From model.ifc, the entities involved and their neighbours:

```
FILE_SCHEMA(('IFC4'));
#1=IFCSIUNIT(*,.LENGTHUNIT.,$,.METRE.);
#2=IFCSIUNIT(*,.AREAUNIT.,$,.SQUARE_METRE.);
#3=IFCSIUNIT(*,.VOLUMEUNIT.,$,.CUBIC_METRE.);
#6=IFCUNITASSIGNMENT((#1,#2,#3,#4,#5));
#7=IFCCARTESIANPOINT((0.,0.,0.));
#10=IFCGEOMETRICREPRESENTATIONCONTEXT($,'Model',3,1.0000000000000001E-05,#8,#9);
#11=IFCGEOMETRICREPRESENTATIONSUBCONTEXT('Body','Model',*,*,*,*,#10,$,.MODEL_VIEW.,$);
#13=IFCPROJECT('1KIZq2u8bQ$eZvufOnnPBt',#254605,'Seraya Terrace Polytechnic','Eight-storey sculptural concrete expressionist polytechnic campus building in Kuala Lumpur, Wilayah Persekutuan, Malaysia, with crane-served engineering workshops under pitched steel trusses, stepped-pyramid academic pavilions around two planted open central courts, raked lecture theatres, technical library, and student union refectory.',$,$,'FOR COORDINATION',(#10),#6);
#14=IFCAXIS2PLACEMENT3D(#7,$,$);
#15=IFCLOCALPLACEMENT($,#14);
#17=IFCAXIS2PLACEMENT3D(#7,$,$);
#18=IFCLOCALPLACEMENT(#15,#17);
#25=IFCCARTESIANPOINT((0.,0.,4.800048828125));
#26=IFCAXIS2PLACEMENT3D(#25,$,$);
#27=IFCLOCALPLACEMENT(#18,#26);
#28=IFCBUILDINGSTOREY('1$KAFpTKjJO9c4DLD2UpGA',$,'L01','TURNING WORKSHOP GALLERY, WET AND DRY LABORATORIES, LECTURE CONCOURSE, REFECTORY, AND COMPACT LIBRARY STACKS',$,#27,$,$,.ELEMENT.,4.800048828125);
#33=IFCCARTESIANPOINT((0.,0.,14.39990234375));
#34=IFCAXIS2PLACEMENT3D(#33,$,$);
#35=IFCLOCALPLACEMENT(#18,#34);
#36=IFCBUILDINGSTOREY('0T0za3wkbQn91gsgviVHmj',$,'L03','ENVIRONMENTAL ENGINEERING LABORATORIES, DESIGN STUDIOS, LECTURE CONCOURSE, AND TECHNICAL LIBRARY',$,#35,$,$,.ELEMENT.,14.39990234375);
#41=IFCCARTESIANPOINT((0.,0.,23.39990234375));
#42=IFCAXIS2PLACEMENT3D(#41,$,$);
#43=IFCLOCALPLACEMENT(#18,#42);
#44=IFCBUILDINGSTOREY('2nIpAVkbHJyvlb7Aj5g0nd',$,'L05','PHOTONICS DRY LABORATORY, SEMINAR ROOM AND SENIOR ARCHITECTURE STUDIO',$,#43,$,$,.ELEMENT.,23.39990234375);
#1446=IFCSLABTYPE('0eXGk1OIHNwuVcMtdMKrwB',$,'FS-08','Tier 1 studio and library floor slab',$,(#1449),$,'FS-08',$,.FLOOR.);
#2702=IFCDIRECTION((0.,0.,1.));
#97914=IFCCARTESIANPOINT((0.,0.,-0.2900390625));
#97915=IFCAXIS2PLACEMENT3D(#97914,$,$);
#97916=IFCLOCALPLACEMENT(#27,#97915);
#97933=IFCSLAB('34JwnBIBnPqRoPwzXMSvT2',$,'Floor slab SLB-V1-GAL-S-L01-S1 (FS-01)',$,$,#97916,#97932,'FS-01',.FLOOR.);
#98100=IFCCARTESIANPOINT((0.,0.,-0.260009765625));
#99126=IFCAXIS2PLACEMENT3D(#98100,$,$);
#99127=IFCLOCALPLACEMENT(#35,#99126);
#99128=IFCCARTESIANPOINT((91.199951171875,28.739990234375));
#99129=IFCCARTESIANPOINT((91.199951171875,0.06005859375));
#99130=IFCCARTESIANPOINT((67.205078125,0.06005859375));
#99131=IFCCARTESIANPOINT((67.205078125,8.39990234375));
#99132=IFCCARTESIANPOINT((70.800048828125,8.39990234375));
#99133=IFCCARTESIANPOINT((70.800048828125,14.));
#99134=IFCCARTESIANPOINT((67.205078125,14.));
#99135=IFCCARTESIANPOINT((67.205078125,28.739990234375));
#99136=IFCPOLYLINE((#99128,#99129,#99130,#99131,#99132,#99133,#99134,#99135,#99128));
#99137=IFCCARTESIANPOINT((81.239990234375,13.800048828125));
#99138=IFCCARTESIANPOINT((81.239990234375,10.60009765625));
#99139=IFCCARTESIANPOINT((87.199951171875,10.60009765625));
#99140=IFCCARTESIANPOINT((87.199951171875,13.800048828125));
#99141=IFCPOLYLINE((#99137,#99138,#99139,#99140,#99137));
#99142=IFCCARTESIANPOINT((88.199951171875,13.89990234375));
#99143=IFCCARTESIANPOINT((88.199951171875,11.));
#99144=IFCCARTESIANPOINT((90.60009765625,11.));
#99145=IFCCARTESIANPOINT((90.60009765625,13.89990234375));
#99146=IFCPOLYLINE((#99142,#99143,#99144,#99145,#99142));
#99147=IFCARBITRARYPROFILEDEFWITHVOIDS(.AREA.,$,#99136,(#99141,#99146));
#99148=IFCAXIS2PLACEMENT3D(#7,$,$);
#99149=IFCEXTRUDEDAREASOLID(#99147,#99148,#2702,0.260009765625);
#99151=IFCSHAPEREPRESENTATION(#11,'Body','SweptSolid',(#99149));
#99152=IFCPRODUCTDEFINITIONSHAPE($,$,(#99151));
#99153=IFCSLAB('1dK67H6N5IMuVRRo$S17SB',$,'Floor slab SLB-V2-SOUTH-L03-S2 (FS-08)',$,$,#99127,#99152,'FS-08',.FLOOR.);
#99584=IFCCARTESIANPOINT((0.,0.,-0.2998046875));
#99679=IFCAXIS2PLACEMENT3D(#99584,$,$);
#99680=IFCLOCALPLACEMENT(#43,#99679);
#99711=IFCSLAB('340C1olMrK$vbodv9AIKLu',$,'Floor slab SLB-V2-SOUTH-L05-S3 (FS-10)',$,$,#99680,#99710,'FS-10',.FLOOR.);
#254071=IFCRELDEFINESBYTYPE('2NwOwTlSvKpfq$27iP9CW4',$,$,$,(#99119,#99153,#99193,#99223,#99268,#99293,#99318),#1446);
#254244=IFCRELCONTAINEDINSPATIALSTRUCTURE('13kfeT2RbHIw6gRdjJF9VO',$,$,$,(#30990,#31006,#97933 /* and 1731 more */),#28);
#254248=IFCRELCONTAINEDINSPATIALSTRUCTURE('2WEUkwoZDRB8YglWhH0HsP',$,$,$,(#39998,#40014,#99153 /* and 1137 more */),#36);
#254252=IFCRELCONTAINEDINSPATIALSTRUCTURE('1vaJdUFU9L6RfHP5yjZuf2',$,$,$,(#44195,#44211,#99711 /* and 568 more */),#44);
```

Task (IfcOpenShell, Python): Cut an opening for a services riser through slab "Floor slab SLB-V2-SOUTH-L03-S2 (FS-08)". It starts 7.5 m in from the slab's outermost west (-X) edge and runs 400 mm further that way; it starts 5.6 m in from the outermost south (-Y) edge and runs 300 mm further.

```python
import numpy as np
import ifcopenshell
import ifcopenshell.api.feature
import ifcopenshell.api.geometry
import ifcopenshell.api.root
import ifcopenshell.geom
import ifcopenshell.util.placement
import ifcopenshell.util.representation
import ifcopenshell.util.shape
import ifcopenshell.util.unit

model = ifcopenshell.open("model.ifc")
unit_scale = ifcopenshell.util.unit.calculate_unit_scale(model)
settings = ifcopenshell.geom.settings()


def volume(element):
    """Net volume in cubic metres, openings subtracted."""
    shape = ifcopenshell.geom.create_shape(settings, element)
    return ifcopenshell.util.shape.get_volume(shape.geometry)


slab = model.by_guid("1dK67H6N5IMuVRRo$S17SB")
before = volume(slab)

# Extent in the slab's own axes, in metres. The edges named are its -X and -Y sides.
slab_shape = ifcopenshell.geom.create_shape(settings, slab)
vertices = ifcopenshell.util.shape.get_vertices(slab_shape.geometry)
x_min, y_min, bottom = vertices.min(axis=0)
top = vertices[:, 2].max()

opening = ifcopenshell.api.root.create_entity(model, ifc_class="IfcOpeningElement", name="Services riser opening", predefined_type="OPENING")
context = ifcopenshell.util.representation.get_context(model, "Model", "Body", "MODEL_VIEW")
width, depth = 0.4, 0.3
outline = [(0.0, 0.0), (width, 0.0), (width, depth), (0.0, depth), (0.0, 0.0)]
# Overshoot both faces by 50 mm so the cut is clean.
shape = ifcopenshell.api.geometry.add_slab_representation(
    model, context=context, depth=top - bottom + 0.1, polyline=outline
)
ifcopenshell.api.geometry.assign_representation(model, product=opening, representation=shape)

matrix = ifcopenshell.util.placement.get_local_placement(slab.ObjectPlacement)
matrix[:, 3] = matrix @ np.append(np.array([x_min + 7.5, y_min + 5.6, bottom - 0.05]) / unit_scale, 1.0)
ifcopenshell.api.geometry.edit_object_placement(model, product=opening, matrix=matrix, is_si=False)
ifcopenshell.api.feature.add_feature(model, feature=opening, element=slab)

after = volume(slab)

print(f"slab volume {before:.3f} -> {after:.3f} m3")

model.write("model_rev.ifc")
```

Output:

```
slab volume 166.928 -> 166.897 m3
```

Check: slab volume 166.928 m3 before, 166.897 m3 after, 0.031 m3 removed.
